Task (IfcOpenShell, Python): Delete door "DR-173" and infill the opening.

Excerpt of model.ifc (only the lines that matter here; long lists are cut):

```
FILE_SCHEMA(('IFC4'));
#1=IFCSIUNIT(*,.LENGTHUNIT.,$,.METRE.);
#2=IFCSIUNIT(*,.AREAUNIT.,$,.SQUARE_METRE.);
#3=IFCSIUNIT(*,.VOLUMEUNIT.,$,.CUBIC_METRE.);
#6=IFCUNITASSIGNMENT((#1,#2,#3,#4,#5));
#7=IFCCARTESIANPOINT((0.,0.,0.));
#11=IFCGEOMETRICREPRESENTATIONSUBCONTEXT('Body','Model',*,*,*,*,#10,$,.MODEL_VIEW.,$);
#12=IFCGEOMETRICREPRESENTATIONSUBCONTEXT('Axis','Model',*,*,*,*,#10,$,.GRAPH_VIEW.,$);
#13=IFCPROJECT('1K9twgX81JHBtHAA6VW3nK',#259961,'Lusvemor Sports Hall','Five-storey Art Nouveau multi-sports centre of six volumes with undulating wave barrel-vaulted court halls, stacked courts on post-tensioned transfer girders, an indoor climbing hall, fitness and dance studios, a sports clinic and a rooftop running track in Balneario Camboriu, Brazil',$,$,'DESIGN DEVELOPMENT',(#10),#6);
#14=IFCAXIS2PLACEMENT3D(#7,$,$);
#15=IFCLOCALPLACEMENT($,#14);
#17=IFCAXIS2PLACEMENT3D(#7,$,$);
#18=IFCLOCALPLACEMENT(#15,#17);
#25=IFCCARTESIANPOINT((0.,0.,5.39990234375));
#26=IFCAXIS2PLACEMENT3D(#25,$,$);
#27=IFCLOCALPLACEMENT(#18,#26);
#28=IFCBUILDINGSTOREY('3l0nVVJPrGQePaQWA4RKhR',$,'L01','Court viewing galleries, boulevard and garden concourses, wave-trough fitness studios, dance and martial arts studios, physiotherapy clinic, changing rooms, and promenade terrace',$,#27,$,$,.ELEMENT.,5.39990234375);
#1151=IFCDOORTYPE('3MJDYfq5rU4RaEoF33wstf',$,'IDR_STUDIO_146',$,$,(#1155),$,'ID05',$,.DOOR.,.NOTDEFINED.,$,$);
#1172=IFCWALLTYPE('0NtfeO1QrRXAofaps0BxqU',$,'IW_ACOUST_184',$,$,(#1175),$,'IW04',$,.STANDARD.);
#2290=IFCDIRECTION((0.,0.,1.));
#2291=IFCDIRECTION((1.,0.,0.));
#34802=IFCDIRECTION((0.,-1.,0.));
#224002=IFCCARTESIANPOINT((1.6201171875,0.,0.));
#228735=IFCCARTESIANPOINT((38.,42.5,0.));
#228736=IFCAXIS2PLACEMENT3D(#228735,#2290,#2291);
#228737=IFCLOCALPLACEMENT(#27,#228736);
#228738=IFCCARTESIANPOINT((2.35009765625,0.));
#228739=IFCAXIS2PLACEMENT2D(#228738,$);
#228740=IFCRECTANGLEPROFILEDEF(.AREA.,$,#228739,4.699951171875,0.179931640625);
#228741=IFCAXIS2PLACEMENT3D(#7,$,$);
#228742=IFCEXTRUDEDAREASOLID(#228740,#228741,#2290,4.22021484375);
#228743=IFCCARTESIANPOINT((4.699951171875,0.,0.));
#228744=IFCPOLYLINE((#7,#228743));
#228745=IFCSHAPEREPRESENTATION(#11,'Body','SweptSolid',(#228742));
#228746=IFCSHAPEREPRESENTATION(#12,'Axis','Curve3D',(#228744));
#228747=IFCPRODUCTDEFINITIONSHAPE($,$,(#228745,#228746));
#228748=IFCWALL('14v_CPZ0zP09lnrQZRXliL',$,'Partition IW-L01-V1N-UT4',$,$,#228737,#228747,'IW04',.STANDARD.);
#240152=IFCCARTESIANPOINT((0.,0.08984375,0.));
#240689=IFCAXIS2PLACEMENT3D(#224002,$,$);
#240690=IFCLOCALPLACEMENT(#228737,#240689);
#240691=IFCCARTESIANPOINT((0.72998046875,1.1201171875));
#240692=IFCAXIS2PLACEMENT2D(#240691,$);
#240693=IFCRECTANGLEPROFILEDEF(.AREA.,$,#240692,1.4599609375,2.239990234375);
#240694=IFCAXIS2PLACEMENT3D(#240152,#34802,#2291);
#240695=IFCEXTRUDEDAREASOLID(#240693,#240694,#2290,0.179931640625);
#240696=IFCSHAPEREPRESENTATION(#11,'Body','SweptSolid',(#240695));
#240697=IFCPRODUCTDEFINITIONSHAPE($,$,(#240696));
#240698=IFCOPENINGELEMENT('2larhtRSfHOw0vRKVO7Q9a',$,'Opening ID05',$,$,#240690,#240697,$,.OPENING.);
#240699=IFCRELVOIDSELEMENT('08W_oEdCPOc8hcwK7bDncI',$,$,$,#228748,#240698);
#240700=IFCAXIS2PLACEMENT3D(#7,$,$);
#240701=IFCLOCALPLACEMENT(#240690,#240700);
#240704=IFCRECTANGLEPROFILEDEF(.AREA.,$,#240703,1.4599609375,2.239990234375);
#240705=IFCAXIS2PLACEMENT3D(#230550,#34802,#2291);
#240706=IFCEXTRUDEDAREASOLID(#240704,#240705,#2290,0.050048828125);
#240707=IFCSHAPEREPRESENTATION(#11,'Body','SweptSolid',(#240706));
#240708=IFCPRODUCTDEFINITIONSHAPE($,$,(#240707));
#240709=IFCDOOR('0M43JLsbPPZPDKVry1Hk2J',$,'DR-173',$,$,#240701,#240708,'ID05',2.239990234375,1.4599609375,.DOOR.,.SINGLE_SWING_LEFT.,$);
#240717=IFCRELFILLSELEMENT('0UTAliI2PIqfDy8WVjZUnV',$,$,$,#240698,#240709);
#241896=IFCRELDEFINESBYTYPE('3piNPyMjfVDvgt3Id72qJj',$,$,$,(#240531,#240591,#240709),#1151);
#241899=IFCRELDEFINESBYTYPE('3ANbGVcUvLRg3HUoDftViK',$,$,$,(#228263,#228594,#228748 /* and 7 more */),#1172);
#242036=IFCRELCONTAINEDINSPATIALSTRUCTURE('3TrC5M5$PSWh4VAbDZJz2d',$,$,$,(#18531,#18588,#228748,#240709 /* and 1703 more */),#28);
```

```python
import ifcopenshell
import ifcopenshell.api.feature
import ifcopenshell.api.root
import ifcopenshell.geom
import ifcopenshell.util.shape

model = ifcopenshell.open("model.ifc")
settings = ifcopenshell.geom.settings()


def volume(element):
    """Net volume in cubic metres, openings subtracted."""
    shape = ifcopenshell.geom.create_shape(settings, element)
    return ifcopenshell.util.shape.get_volume(shape.geometry)


door = model.by_guid("0M43JLsbPPZPDKVry1Hk2J")
opening = door.FillsVoids[0].RelatingOpeningElement
wall = opening.VoidsElements[0].RelatingBuildingElement
before = volume(wall)

ifcopenshell.api.root.remove_product(model, product=door)
ifcopenshell.api.feature.remove_feature(model, feature=opening)

after = volume(wall)

print(f"wall volume {before:.3f} -> {after:.3f} m3")

model.write("model_rev.ifc")
```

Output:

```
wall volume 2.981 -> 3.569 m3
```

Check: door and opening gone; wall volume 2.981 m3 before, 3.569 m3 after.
